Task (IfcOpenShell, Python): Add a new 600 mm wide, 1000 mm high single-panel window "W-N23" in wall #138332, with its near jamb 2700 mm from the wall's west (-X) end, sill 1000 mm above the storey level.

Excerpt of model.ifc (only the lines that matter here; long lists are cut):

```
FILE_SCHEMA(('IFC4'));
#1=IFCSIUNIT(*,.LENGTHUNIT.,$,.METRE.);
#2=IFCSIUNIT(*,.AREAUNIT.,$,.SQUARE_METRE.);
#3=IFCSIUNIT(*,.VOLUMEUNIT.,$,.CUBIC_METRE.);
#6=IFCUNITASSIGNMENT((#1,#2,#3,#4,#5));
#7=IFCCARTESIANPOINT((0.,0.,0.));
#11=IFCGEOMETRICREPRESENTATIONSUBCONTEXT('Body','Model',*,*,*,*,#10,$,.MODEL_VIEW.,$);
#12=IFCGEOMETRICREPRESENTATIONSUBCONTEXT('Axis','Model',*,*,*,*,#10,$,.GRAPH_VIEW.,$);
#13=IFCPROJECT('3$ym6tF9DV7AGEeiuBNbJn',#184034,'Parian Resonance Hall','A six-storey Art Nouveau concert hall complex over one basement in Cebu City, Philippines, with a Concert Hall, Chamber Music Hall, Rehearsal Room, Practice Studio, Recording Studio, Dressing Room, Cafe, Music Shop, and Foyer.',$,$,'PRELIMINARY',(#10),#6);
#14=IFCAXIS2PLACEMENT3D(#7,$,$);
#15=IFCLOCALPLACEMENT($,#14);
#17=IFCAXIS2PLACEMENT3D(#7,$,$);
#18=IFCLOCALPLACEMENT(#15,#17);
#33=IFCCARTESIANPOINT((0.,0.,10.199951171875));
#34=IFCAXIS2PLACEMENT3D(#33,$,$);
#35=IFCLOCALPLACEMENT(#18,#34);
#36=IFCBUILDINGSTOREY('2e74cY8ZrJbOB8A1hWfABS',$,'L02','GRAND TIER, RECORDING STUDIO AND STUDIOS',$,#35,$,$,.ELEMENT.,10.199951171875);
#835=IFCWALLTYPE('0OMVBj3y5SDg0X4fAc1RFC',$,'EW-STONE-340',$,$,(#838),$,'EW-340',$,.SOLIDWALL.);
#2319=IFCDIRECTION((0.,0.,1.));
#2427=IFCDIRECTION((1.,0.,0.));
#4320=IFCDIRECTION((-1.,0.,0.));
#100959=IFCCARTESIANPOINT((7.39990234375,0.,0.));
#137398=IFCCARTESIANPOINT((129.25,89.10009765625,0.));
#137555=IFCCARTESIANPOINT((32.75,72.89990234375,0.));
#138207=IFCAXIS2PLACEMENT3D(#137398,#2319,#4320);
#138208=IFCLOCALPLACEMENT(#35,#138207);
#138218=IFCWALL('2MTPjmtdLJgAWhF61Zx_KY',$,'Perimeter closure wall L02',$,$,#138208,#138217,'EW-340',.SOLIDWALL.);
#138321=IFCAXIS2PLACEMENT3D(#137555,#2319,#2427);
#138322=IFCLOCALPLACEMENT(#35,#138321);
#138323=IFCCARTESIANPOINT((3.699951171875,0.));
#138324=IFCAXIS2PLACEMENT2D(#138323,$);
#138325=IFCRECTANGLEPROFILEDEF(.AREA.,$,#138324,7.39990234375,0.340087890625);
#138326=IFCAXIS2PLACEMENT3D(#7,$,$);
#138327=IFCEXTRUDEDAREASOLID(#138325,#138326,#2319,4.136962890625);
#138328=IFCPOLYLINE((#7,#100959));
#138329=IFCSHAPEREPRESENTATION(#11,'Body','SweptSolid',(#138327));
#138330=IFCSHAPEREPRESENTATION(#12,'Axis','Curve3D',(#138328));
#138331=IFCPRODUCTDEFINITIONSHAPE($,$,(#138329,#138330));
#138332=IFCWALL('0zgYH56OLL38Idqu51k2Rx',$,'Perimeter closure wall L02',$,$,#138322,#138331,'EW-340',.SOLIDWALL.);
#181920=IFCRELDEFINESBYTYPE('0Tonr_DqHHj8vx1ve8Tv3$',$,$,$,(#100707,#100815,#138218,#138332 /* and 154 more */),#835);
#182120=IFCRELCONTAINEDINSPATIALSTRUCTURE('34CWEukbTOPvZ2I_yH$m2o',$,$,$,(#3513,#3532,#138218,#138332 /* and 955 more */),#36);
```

```python
import numpy as np
import ifcopenshell
import ifcopenshell.api.feature
import ifcopenshell.api.geometry
import ifcopenshell.api.root
import ifcopenshell.api.spatial
import ifcopenshell.geom
import ifcopenshell.util.element
import ifcopenshell.util.placement
import ifcopenshell.util.representation
import ifcopenshell.util.shape
import ifcopenshell.util.unit

model = ifcopenshell.open("model.ifc")
unit_scale = ifcopenshell.util.unit.calculate_unit_scale(model)
settings = ifcopenshell.geom.settings()


def volume(element):
    """Net volume in cubic metres, openings subtracted."""
    shape = ifcopenshell.geom.create_shape(settings, element)
    return ifcopenshell.util.shape.get_volume(shape.geometry)


wall = model.by_id(138332)
storey = ifcopenshell.util.element.get_container(wall, ifc_class="IfcBuildingStorey")
context = ifcopenshell.util.representation.get_context(model, "Model", "Body", "MODEL_VIEW")
before = volume(wall)

width, height, from_end, sill = 0.6, 1, 2.7, 1  # metres

# The wall runs along its own X axis, and the end named is its -X end.
wall_shape = ifcopenshell.geom.create_shape(settings, wall)
x, y, z = ifcopenshell.util.shape.get_vertices(wall_shape.geometry).T
start = x.min() + from_end
face, thickness = float(y.min()), float(y.max() - y.min())
wall_matrix = ifcopenshell.util.placement.get_local_placement(wall.ObjectPlacement)
level = ifcopenshell.util.placement.get_local_placement(storey.ObjectPlacement)[2, 3]


def in_wall(x, y):
    """Placement at x, y metres in the wall's axes, at sill height."""
    matrix = wall_matrix.copy()
    matrix[:, 3] = wall_matrix @ np.array([x / unit_scale, y / unit_scale, 0.0, 1.0])
    matrix[2, 3] = level + sill / unit_scale
    return matrix


# Opening: a box that overshoots both wall faces by 50 mm.
opening = ifcopenshell.api.root.create_entity(model, ifc_class="IfcOpeningElement", predefined_type="OPENING")
box = ifcopenshell.api.geometry.add_wall_representation(
    model, context=context, length=width, height=height, thickness=thickness + 0.1
)
ifcopenshell.api.geometry.assign_representation(model, product=opening, representation=box)
ifcopenshell.api.geometry.edit_object_placement(model, product=opening, matrix=in_wall(start, face - 0.05), is_si=False)
ifcopenshell.api.feature.add_feature(model, feature=opening, element=wall)

window = ifcopenshell.api.root.create_entity(model, ifc_class="IfcWindow", name="W-N23", predefined_type="WINDOW")
window.OverallWidth, window.OverallHeight = width / unit_scale, height / unit_scale
window.PartitioningType = "SINGLE_PANEL"
body = ifcopenshell.api.geometry.add_window_representation(
    model,
    context=context,
    overall_width=window.OverallWidth,
    overall_height=window.OverallHeight,
    partition_type="SINGLE_PANEL",
)
ifcopenshell.api.geometry.assign_representation(model, product=window, representation=body)
ifcopenshell.api.spatial.assign_container(model, products=[window], relating_structure=storey)
ifcopenshell.api.feature.add_filling(model, opening=opening, element=window)

# Centre the window in the wall's thickness.
ifcopenshell.api.geometry.edit_object_placement(model, product=window, matrix=in_wall(start, face), is_si=False)
window_shape = ifcopenshell.geom.create_shape(settings, window)
depth = ifcopenshell.util.shape.get_vertices(window_shape.geometry)[:, 1]
offset = face + thickness / 2 - (depth.min() + depth.max()) / 2
ifcopenshell.api.geometry.edit_object_placement(model, product=window, matrix=in_wall(start, offset), is_si=False)

after = volume(wall)

print(f"wall volume {before:.3f} -> {after:.3f} m3")

model.write("model_v2.ifc")
```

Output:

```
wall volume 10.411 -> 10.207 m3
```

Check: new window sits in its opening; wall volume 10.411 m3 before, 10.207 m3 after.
